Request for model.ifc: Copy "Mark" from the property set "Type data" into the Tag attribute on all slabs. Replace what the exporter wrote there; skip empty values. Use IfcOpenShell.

First a look at what the model holds.

```python
import ifcopenshell
import ifcopenshell.util.element

model = ifcopenshell.open("model.ifc")
print(model.schema)
slabs = model.by_type("IfcSlab")
print(len(slabs), "slabs")
for e in slabs[:8]:
    source = ifcopenshell.util.element.get_pset(e, "Type data", "Mark")
    target = e.Tag
    print(e.id(), repr(source), repr(target), sep=" | ")
```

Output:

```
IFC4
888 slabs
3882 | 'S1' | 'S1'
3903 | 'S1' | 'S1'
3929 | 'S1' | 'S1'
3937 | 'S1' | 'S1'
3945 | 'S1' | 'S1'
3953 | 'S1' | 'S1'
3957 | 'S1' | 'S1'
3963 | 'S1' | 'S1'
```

```python
import ifcopenshell
import ifcopenshell.util.element

model = ifcopenshell.open("model.ifc")

count = 0
for e in model.by_type("IfcSlab"):
    value = ifcopenshell.util.element.get_pset(e, "Type data", "Mark")
    current = e.Tag
    if not value or not value.strip() or current == value:
        continue
    e.Tag = value
    count += 1

print(count, "slabs updated")

model.write("model_updated.ifc")
```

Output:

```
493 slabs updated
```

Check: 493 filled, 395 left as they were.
